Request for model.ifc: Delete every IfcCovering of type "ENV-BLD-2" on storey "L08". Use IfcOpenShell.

First a look at what the model holds.

```python
import ifcopenshell
import ifcopenshell.util.element

model = ifcopenshell.open("model.ifc")
print(model.schema)
storey = next(s for s in model.by_type("IfcBuildingStorey") if s.Name == "L08")
coverings = [e for e in ifcopenshell.util.element.get_decomposition(storey) if e.is_a("IfcCovering")]
seen = {}
for e in coverings:
    element_type = ifcopenshell.util.element.get_type(e)
    name = element_type.Name if element_type not in (None, e) else None
    seen[name] = seen.get(name, 0) + 1
for name, count in sorted(seen.items(), key=str):
    print(count, "x", name)
```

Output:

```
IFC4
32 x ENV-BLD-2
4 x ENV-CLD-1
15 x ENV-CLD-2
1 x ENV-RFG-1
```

```python
import ifcopenshell
import ifcopenshell.api.root
import ifcopenshell.util.element

model = ifcopenshell.open("model.ifc")

storey = next(s for s in model.by_type("IfcBuildingStorey") if s.Name == "L08")
coverings = [e for e in ifcopenshell.util.element.get_decomposition(storey) if e.is_a("IfcCovering")]
targets = [e for e in coverings if (t := ifcopenshell.util.element.get_type(e)) not in (None, e) and t.Name == "ENV-BLD-2"]

for e in targets:
    ifcopenshell.api.root.remove_product(model, product=e)
print(len(targets), "removed")

model.write("model_updated.ifc")
```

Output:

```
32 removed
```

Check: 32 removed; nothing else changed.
